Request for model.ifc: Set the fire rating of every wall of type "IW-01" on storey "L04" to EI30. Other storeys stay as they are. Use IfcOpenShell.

First a look at what the model holds.

```python
import ifcopenshell
import ifcopenshell.util.element

model = ifcopenshell.open("model.ifc")
print(model.schema)
storey = next(s for s in model.by_type("IfcBuildingStorey") if s.Name == "L04")
walls = [e for e in ifcopenshell.util.element.get_decomposition(storey) if e.is_a("IfcWall")]
seen = {}
for e in walls:
    element_type = ifcopenshell.util.element.get_type(e)
    key = (element_type.Name if element_type != e and element_type else None, ifcopenshell.util.element.get_pset(e, "Pset_WallCommon", "FireRating"))
    seen[key] = seen.get(key, 0) + 1
for (name, value), count in sorted(seen.items(), key=str):
    print(count, "x", name, "|", value)
```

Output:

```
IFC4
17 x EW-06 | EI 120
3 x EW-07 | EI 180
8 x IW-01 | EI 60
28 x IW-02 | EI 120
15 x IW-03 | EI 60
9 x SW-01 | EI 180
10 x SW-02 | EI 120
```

```python
import ifcopenshell
import ifcopenshell.api.pset
import ifcopenshell.util.element

model = ifcopenshell.open("model.ifc")

storey = next(s for s in model.by_type("IfcBuildingStorey") if s.Name == "L04")
walls = [e for e in ifcopenshell.util.element.get_decomposition(storey) if e.is_a("IfcWall")]

count = 0
for e in walls:
    element_type = ifcopenshell.util.element.get_type(e)
    if element_type in (None, e) or element_type.Name != "IW-01":
        continue
    # add_pset returns the element's existing set when there is one.
    pset = ifcopenshell.api.pset.add_pset(model, product=e, name="Pset_WallCommon")
    ifcopenshell.api.pset.edit_pset(model, pset=pset, properties={"FireRating": "EI30"})
    count += 1

print(count, "walls updated")

model.write("model_edited.ifc")
```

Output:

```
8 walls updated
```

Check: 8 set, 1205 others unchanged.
